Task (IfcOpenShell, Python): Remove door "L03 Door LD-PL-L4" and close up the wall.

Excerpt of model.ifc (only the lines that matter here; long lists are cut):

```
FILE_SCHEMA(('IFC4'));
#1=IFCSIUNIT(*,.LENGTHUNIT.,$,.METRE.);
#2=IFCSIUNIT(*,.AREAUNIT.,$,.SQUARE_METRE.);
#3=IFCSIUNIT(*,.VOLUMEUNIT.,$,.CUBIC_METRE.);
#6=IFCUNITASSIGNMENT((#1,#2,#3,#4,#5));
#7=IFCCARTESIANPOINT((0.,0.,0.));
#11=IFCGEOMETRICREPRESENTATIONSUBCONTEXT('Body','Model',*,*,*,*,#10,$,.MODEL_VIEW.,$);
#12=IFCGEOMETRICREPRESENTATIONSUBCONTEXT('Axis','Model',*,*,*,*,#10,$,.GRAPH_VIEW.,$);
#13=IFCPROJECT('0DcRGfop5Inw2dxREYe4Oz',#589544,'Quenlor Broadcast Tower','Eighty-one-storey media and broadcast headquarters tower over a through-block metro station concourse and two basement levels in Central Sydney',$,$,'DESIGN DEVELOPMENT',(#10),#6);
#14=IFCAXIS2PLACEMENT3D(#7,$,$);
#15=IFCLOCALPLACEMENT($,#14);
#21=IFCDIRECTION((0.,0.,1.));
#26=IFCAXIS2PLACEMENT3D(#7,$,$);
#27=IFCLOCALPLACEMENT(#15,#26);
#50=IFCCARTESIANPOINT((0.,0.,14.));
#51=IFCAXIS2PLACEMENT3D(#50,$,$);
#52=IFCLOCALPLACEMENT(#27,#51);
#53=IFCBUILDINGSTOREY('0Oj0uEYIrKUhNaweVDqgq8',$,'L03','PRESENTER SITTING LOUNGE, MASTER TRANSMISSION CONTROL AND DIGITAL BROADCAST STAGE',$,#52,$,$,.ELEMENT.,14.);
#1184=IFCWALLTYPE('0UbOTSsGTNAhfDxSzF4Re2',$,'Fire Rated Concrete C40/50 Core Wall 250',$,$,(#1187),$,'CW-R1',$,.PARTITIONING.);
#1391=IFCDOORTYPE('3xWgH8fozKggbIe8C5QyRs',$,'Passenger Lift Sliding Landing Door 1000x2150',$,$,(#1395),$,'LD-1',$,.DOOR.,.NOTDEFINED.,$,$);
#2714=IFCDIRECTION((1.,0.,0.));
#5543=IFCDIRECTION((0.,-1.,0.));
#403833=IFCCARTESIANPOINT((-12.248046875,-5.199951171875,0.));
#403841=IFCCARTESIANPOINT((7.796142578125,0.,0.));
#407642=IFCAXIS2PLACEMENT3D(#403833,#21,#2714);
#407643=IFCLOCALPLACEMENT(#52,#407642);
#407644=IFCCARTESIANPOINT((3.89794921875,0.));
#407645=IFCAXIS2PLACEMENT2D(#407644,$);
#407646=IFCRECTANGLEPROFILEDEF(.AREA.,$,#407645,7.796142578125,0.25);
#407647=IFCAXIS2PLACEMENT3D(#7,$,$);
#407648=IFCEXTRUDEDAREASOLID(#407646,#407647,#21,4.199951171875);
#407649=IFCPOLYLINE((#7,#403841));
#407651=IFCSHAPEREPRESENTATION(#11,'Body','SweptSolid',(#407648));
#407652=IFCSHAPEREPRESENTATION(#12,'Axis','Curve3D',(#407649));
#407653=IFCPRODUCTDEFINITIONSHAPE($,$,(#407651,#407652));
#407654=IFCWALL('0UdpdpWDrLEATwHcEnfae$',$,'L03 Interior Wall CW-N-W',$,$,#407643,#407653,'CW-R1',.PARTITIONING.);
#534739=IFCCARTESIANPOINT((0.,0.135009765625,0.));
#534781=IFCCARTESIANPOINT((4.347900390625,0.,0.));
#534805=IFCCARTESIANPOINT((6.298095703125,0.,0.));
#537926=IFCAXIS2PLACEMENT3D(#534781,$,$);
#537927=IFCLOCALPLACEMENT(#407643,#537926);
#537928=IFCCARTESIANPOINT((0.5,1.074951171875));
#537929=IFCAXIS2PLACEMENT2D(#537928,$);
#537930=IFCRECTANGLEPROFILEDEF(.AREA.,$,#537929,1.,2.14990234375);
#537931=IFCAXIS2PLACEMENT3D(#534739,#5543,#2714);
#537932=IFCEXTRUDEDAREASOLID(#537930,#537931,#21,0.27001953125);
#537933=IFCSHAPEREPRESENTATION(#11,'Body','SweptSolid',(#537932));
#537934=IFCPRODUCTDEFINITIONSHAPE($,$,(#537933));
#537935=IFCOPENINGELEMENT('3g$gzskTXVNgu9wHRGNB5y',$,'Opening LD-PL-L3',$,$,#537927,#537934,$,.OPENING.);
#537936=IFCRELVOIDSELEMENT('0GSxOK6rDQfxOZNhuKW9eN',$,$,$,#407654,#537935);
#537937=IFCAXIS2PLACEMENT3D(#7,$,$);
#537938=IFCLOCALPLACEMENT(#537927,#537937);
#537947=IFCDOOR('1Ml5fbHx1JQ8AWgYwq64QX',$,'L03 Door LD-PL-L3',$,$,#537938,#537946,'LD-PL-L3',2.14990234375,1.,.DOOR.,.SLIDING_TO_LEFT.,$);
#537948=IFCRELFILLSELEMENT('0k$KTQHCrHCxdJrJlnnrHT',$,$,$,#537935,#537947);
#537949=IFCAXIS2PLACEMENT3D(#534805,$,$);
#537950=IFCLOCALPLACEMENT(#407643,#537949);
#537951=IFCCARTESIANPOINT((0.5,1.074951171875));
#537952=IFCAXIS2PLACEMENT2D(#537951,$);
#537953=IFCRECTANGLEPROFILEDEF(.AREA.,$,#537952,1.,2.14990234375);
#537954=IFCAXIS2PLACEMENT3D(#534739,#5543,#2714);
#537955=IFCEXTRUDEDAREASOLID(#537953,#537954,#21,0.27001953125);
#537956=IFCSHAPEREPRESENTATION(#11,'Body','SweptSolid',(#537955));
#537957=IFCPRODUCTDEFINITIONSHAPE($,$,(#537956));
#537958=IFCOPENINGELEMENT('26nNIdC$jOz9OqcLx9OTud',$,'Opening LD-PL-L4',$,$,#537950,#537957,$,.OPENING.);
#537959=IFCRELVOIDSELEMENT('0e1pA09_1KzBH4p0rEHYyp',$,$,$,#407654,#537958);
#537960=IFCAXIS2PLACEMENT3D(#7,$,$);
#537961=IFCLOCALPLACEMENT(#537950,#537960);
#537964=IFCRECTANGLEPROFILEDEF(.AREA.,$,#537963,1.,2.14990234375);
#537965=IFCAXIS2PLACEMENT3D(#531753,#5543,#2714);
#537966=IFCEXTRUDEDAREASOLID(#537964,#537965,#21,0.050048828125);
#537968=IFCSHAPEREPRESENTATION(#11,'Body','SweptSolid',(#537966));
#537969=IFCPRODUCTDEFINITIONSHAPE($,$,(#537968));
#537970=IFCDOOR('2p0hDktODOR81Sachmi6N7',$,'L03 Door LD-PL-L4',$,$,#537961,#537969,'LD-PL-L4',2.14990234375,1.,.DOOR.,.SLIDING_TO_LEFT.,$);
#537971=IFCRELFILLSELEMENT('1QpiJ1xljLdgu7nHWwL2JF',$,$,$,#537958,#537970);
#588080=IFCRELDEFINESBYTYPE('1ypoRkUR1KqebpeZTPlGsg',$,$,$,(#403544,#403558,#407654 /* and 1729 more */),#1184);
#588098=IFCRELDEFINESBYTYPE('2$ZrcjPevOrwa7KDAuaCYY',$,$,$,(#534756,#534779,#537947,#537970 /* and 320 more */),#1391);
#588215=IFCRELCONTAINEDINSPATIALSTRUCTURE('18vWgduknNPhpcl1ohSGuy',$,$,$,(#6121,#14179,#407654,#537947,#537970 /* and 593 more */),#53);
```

```python
import ifcopenshell
import ifcopenshell.api.feature
import ifcopenshell.api.root
import ifcopenshell.geom
import ifcopenshell.util.shape

model = ifcopenshell.open("model.ifc")
settings = ifcopenshell.geom.settings()


def volume(element):
    """Net volume in cubic metres, openings subtracted."""
    shape = ifcopenshell.geom.create_shape(settings, element)
    return ifcopenshell.util.shape.get_volume(shape.geometry)


door = model.by_guid("2p0hDktODOR81Sachmi6N7")
opening = door.FillsVoids[0].RelatingOpeningElement
wall = opening.VoidsElements[0].RelatingBuildingElement
before = volume(wall)

ifcopenshell.api.root.remove_product(model, product=door)
ifcopenshell.api.feature.remove_feature(model, feature=opening)

after = volume(wall)

print(f"wall volume {before:.3f} -> {after:.3f} m3")

model.write("model_edited.ifc")
```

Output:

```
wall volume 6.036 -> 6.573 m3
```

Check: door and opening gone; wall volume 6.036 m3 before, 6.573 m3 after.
